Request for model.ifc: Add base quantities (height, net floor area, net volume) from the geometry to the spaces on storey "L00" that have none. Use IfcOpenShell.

First a look at what the model holds.

```python
import ifcopenshell
import ifcopenshell.util.element
import ifcopenshell.util.unit

model = ifcopenshell.open("model.ifc")
print(model.schema)
for unit_type in ("LENGTHUNIT", "AREAUNIT", "VOLUMEUNIT"):
    print(unit_type, ifcopenshell.util.unit.calculate_unit_scale(model, unit_type))
storey = next(s for s in model.by_type("IfcBuildingStorey") if s.Name == "L00")
spaces = [e for e in ifcopenshell.util.element.get_decomposition(storey) if e.is_a("IfcSpace")]
for e in sorted(spaces, key=lambda e: e.id()):
    print(e.id(), e.is_a(), e.Name, list(ifcopenshell.util.element.get_psets(e, qtos_only=True)), sep=" | ")
```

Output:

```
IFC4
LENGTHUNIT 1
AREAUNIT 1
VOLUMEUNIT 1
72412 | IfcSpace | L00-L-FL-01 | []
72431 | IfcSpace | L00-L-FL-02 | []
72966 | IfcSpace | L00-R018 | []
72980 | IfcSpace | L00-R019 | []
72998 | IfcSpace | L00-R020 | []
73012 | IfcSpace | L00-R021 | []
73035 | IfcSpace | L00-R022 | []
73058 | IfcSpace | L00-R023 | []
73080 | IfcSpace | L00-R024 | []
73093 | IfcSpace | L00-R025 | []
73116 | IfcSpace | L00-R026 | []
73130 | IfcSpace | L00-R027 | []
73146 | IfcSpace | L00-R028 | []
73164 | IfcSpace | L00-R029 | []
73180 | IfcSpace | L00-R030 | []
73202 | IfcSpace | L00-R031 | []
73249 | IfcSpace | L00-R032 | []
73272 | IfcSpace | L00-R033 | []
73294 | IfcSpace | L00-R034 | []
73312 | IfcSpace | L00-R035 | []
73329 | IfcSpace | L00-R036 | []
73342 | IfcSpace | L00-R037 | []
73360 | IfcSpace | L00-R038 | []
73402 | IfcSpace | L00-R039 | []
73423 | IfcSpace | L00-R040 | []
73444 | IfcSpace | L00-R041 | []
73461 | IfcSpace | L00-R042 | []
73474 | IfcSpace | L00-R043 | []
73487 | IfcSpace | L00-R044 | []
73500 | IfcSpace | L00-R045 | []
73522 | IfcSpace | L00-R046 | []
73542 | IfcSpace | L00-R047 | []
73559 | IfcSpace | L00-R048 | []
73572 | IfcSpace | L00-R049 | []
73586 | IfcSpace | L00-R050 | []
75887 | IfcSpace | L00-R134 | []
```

```python
import ifcopenshell
import ifcopenshell.api.pset
import ifcopenshell.geom
import ifcopenshell.util.element
import ifcopenshell.util.shape
import ifcopenshell.util.unit

model = ifcopenshell.open("model.ifc")
unit_scale = ifcopenshell.util.unit.calculate_unit_scale(model)
area_scale = ifcopenshell.util.unit.calculate_unit_scale(model, "AREAUNIT")
volume_scale = ifcopenshell.util.unit.calculate_unit_scale(model, "VOLUMEUNIT")
settings = ifcopenshell.geom.settings()

storey = next(s for s in model.by_type("IfcBuildingStorey") if s.Name == "L00")
spaces = [e for e in ifcopenshell.util.element.get_decomposition(storey) if e.is_a("IfcSpace")]

for e in sorted(spaces, key=lambda e: e.id()):
    if ifcopenshell.util.element.get_psets(e, qtos_only=True, should_inherit=False):
        continue
    # Geometry comes back in metres, in the element's own axes.
    shape = ifcopenshell.geom.create_shape(settings, e)
    values = {
        "Height": ifcopenshell.util.shape.get_z(shape.geometry) / unit_scale,
        "NetFloorArea": ifcopenshell.util.shape.get_footprint_area(shape.geometry) / area_scale,
        "NetVolume": ifcopenshell.util.shape.get_volume(shape.geometry) / volume_scale,
    }
    qto = ifcopenshell.api.pset.add_qto(model, product=e, name="Qto_SpaceBaseQuantities")
    ifcopenshell.api.pset.edit_qto(model, qto=qto, properties=values)
    print(e.id(), {k: round(v, 3) for k, v in values.items()})

model.write("model_v2.ifc")
```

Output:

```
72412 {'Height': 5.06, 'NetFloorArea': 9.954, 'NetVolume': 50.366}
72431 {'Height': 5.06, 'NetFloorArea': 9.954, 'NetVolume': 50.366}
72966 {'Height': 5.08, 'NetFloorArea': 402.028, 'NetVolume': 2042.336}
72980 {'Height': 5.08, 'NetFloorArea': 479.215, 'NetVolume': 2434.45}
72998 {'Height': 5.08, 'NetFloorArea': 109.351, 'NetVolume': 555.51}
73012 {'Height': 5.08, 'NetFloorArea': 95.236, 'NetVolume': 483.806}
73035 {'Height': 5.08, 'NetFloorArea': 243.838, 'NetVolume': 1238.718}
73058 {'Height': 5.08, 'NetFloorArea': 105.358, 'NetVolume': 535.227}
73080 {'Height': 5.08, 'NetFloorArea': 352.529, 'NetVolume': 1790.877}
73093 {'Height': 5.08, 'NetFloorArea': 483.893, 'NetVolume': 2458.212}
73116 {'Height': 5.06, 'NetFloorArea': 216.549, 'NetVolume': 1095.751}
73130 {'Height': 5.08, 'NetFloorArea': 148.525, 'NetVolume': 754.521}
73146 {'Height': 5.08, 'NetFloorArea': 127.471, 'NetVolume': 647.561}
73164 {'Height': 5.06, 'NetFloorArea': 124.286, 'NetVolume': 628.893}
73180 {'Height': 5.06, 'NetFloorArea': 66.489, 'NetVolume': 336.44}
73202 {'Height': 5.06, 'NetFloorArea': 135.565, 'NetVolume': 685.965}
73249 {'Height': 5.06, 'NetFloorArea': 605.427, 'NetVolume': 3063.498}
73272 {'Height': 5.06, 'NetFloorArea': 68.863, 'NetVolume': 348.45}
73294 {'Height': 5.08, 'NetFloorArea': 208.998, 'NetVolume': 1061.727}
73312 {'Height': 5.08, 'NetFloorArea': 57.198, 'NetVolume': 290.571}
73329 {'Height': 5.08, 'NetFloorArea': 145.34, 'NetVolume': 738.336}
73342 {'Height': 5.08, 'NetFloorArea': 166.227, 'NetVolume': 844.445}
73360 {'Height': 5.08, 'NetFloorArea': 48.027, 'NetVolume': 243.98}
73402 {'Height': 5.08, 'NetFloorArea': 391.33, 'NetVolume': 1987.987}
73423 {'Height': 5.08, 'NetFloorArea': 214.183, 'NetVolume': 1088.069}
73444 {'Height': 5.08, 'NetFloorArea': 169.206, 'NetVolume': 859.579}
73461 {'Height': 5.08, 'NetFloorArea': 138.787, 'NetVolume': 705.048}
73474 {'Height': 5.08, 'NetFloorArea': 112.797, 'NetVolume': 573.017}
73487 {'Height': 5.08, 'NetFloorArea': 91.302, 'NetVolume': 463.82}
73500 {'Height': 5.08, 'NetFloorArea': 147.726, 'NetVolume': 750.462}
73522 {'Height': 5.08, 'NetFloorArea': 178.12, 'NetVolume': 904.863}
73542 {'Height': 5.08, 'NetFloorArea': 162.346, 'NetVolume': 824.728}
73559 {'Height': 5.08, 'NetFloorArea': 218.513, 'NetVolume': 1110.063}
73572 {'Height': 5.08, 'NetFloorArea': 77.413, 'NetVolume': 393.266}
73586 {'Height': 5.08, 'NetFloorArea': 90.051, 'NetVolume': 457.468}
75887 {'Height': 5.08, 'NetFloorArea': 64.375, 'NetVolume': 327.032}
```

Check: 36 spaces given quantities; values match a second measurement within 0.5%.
